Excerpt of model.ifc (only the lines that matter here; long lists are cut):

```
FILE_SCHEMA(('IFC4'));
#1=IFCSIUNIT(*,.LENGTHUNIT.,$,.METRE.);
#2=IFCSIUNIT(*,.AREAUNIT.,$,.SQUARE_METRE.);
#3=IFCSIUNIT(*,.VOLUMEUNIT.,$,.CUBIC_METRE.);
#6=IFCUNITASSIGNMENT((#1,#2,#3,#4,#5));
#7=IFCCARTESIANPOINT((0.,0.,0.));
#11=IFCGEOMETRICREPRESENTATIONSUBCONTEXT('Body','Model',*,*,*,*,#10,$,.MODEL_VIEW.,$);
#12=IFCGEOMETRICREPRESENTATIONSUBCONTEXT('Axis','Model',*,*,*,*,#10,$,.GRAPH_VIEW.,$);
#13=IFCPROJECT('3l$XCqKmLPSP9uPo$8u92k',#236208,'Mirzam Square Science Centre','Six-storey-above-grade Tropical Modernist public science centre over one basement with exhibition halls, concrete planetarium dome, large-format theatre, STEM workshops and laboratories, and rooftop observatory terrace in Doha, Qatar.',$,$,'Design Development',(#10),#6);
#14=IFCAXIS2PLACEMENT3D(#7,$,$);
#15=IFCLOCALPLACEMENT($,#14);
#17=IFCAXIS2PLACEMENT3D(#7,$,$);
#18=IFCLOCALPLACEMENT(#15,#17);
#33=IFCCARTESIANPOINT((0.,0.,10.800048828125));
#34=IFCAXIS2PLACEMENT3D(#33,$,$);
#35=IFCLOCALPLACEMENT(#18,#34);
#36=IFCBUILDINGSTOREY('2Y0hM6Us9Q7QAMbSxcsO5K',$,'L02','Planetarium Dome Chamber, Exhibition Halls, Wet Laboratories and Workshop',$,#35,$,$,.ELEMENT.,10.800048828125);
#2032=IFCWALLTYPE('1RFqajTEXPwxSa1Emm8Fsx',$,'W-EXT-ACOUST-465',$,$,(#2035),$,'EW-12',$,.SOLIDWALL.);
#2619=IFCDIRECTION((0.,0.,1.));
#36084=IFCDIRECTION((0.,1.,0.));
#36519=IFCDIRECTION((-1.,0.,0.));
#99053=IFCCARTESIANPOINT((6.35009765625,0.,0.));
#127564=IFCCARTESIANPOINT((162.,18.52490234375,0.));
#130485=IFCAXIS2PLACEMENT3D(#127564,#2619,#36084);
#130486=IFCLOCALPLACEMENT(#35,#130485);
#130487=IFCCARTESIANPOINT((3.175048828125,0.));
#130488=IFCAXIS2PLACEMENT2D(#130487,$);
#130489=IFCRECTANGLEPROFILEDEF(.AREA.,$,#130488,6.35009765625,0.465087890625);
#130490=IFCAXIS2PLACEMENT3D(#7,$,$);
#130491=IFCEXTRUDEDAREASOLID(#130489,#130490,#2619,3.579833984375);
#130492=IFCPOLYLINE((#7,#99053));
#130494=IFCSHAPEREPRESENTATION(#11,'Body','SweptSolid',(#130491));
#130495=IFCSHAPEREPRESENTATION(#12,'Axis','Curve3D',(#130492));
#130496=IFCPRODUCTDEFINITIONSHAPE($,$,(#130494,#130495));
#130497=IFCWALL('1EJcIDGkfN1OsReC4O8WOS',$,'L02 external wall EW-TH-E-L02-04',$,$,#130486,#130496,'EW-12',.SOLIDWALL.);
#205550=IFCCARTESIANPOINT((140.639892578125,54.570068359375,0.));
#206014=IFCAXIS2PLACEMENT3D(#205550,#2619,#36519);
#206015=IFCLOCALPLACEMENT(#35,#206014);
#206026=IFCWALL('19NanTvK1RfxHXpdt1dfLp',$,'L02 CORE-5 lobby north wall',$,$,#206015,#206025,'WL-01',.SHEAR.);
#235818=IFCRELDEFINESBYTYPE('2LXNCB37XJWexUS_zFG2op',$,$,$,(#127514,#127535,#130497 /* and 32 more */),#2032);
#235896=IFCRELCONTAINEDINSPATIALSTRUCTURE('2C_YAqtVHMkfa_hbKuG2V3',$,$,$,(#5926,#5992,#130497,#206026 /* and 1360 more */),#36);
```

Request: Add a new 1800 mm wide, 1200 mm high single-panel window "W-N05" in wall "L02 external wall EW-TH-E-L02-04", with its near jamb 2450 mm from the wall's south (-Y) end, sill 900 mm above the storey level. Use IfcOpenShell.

```python
import numpy as np
import ifcopenshell
import ifcopenshell.api.feature
import ifcopenshell.api.geometry
import ifcopenshell.api.root
import ifcopenshell.api.spatial
import ifcopenshell.geom
import ifcopenshell.util.element
import ifcopenshell.util.placement
import ifcopenshell.util.representation
import ifcopenshell.util.shape
import ifcopenshell.util.unit

model = ifcopenshell.open("model.ifc")
unit_scale = ifcopenshell.util.unit.calculate_unit_scale(model)
settings = ifcopenshell.geom.settings()


def volume(element):
    """Net volume in cubic metres, openings subtracted."""
    shape = ifcopenshell.geom.create_shape(settings, element)
    return ifcopenshell.util.shape.get_volume(shape.geometry)


wall = model.by_id(130497)
storey = ifcopenshell.util.element.get_container(wall, ifc_class="IfcBuildingStorey")
context = ifcopenshell.util.representation.get_context(model, "Model", "Body", "MODEL_VIEW")
before = volume(wall)

width, height, from_end, sill = 1.8, 1.2, 2.45, 0.9  # metres

# The wall runs along its own X axis, and the end named is its -X end.
wall_shape = ifcopenshell.geom.create_shape(settings, wall)
x, y, z = ifcopenshell.util.shape.get_vertices(wall_shape.geometry).T
start = x.min() + from_end
face, thickness = float(y.min()), float(y.max() - y.min())
wall_matrix = ifcopenshell.util.placement.get_local_placement(wall.ObjectPlacement)
level = ifcopenshell.util.placement.get_local_placement(storey.ObjectPlacement)[2, 3]


def in_wall(x, y):
    """Placement at x, y metres in the wall's axes, at sill height."""
    matrix = wall_matrix.copy()
    matrix[:, 3] = wall_matrix @ np.array([x / unit_scale, y / unit_scale, 0.0, 1.0])
    matrix[2, 3] = level + sill / unit_scale
    return matrix


# Opening: a box that overshoots both wall faces by 50 mm.
opening = ifcopenshell.api.root.create_entity(model, ifc_class="IfcOpeningElement", predefined_type="OPENING")
box = ifcopenshell.api.geometry.add_wall_representation(
    model, context=context, length=width, height=height, thickness=thickness + 0.1
)
ifcopenshell.api.geometry.assign_representation(model, product=opening, representation=box)
ifcopenshell.api.geometry.edit_object_placement(model, product=opening, matrix=in_wall(start, face - 0.05), is_si=False)
ifcopenshell.api.feature.add_feature(model, feature=opening, element=wall)

window = ifcopenshell.api.root.create_entity(model, ifc_class="IfcWindow", name="W-N05", predefined_type="WINDOW")
window.OverallWidth, window.OverallHeight = width / unit_scale, height / unit_scale
window.PartitioningType = "SINGLE_PANEL"
body = ifcopenshell.api.geometry.add_window_representation(
    model,
    context=context,
    overall_width=window.OverallWidth,
    overall_height=window.OverallHeight,
    partition_type="SINGLE_PANEL",
)
ifcopenshell.api.geometry.assign_representation(model, product=window, representation=body)
ifcopenshell.api.spatial.assign_container(model, products=[window], relating_structure=storey)
ifcopenshell.api.feature.add_filling(model, opening=opening, element=window)

# Centre the window in the wall's thickness.
ifcopenshell.api.geometry.edit_object_placement(model, product=window, matrix=in_wall(start, face), is_si=False)
window_shape = ifcopenshell.geom.create_shape(settings, window)
depth = ifcopenshell.util.shape.get_vertices(window_shape.geometry)[:, 1]
offset = face + thickness / 2 - (depth.min() + depth.max()) / 2
ifcopenshell.api.geometry.edit_object_placement(model, product=window, matrix=in_wall(start, offset), is_si=False)

after = volume(wall)

print(f"wall volume {before:.3f} -> {after:.3f} m3")

model.write("model-out.ifc")
```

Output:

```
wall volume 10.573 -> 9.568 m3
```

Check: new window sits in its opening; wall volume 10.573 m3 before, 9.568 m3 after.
